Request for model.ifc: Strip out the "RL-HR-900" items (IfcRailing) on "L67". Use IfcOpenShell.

First a look at what the model holds.

```python
import ifcopenshell
import ifcopenshell.util.element

model = ifcopenshell.open("model.ifc")
print(model.schema)
storey = next(s for s in model.by_type("IfcBuildingStorey") if s.Name == "L67")
railings = [e for e in ifcopenshell.util.element.get_decomposition(storey) if e.is_a("IfcRailing")]
seen = {}
for e in railings:
    element_type = ifcopenshell.util.element.get_type(e)
    name = element_type.Name if element_type not in (None, e) else None
    seen[name] = seen.get(name, 0) + 1
for name, count in sorted(seen.items(), key=str):
    print(count, "x", name)
```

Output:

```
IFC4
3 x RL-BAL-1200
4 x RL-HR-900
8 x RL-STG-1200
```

```python
import ifcopenshell
import ifcopenshell.api.root
import ifcopenshell.util.element

model = ifcopenshell.open("model.ifc")

storey = next(s for s in model.by_type("IfcBuildingStorey") if s.Name == "L67")
railings = [e for e in ifcopenshell.util.element.get_decomposition(storey) if e.is_a("IfcRailing")]
targets = [e for e in railings if (t := ifcopenshell.util.element.get_type(e)) not in (None, e) and t.Name == "RL-HR-900"]

for e in targets:
    ifcopenshell.api.root.remove_product(model, product=e)
print(len(targets), "removed")

model.write("model_rev.ifc")
```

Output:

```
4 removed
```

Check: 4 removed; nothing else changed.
